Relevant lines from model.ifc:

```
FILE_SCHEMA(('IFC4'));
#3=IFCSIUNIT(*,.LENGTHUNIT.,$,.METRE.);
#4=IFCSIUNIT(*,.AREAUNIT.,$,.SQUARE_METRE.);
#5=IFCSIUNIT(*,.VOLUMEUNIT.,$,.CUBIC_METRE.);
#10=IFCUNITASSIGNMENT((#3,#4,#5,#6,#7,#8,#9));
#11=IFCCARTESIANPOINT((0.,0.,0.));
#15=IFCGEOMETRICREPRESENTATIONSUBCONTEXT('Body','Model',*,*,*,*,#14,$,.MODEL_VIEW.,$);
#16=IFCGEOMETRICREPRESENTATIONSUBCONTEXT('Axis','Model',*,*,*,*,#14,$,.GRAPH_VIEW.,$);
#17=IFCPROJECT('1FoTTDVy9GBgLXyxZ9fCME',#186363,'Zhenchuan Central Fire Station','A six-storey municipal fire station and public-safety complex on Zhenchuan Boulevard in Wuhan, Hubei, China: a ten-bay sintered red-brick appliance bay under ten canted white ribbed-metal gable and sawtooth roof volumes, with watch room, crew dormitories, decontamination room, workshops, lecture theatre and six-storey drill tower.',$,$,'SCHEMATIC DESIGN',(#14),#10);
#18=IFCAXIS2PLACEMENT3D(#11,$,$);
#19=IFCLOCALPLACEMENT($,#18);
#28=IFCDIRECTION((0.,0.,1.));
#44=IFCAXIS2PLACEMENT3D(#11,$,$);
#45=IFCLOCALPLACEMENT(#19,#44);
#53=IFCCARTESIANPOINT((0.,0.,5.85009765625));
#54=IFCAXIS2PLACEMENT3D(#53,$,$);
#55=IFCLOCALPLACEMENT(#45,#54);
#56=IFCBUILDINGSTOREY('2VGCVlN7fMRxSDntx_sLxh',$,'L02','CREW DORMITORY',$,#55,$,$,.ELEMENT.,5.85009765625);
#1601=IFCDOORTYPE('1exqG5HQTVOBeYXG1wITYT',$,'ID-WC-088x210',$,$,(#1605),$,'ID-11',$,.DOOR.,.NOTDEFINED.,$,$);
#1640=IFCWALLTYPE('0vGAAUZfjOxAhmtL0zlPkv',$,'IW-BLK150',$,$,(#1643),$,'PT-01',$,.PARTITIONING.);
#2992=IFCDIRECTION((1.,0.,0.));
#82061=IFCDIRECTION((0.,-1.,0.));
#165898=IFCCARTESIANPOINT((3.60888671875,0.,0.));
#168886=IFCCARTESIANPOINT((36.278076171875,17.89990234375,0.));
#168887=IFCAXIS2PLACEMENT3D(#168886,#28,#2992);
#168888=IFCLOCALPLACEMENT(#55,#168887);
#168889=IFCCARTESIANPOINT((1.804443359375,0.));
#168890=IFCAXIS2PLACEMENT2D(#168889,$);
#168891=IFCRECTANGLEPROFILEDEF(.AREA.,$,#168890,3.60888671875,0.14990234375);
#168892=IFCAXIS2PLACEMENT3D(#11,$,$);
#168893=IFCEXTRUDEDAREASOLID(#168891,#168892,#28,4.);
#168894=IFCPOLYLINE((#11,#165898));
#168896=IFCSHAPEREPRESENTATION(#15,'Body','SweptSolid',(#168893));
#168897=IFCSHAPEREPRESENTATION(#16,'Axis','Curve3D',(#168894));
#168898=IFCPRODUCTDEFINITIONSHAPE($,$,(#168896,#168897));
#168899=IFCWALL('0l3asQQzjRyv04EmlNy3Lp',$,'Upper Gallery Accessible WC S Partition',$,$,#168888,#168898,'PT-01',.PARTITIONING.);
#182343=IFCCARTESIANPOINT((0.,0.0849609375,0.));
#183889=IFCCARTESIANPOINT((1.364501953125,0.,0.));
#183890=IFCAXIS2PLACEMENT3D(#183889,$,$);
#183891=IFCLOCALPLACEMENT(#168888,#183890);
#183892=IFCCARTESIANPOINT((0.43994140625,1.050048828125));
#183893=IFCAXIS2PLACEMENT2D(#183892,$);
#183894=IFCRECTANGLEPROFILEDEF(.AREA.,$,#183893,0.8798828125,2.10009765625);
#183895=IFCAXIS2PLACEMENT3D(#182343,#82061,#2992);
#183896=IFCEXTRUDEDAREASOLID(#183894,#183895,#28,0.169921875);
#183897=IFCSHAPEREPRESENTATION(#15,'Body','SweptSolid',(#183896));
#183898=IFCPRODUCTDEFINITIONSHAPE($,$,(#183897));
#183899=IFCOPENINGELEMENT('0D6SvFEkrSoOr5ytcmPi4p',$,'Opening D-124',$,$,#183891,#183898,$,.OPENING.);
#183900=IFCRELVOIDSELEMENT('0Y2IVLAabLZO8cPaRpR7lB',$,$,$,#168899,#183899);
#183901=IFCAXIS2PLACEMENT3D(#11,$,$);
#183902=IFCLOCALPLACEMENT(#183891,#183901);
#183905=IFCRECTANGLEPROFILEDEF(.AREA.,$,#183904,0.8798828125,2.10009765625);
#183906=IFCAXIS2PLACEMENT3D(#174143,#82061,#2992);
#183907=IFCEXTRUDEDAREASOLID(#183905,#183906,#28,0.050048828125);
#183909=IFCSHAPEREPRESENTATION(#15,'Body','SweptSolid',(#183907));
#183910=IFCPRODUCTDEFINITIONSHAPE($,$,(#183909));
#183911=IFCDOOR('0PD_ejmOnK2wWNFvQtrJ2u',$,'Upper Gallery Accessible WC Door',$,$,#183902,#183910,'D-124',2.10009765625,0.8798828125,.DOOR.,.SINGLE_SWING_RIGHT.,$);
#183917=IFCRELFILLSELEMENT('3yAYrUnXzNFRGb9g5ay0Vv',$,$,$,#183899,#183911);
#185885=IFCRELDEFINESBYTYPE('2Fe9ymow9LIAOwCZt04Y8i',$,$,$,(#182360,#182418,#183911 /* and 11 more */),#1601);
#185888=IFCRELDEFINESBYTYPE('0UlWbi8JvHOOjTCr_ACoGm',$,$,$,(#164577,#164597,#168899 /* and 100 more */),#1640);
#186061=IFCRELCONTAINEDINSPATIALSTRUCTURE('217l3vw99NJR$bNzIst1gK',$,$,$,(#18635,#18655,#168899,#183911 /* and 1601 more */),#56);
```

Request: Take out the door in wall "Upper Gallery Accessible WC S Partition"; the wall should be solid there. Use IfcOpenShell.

```python
import ifcopenshell
import ifcopenshell.api.feature
import ifcopenshell.api.root
import ifcopenshell.geom
import ifcopenshell.util.shape

model = ifcopenshell.open("model.ifc")
settings = ifcopenshell.geom.settings()


def volume(element):
    """Net volume in cubic metres, openings subtracted."""
    shape = ifcopenshell.geom.create_shape(settings, element)
    return ifcopenshell.util.shape.get_volume(shape.geometry)


door = model.by_guid("0PD_ejmOnK2wWNFvQtrJ2u")
opening = door.FillsVoids[0].RelatingOpeningElement
wall = opening.VoidsElements[0].RelatingBuildingElement
before = volume(wall)

ifcopenshell.api.root.remove_product(model, product=door)
ifcopenshell.api.feature.remove_feature(model, feature=opening)

after = volume(wall)

print(f"wall volume {before:.3f} -> {after:.3f} m3")

model.write("model-out.ifc")
```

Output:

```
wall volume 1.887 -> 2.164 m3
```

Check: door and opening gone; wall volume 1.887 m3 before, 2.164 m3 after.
